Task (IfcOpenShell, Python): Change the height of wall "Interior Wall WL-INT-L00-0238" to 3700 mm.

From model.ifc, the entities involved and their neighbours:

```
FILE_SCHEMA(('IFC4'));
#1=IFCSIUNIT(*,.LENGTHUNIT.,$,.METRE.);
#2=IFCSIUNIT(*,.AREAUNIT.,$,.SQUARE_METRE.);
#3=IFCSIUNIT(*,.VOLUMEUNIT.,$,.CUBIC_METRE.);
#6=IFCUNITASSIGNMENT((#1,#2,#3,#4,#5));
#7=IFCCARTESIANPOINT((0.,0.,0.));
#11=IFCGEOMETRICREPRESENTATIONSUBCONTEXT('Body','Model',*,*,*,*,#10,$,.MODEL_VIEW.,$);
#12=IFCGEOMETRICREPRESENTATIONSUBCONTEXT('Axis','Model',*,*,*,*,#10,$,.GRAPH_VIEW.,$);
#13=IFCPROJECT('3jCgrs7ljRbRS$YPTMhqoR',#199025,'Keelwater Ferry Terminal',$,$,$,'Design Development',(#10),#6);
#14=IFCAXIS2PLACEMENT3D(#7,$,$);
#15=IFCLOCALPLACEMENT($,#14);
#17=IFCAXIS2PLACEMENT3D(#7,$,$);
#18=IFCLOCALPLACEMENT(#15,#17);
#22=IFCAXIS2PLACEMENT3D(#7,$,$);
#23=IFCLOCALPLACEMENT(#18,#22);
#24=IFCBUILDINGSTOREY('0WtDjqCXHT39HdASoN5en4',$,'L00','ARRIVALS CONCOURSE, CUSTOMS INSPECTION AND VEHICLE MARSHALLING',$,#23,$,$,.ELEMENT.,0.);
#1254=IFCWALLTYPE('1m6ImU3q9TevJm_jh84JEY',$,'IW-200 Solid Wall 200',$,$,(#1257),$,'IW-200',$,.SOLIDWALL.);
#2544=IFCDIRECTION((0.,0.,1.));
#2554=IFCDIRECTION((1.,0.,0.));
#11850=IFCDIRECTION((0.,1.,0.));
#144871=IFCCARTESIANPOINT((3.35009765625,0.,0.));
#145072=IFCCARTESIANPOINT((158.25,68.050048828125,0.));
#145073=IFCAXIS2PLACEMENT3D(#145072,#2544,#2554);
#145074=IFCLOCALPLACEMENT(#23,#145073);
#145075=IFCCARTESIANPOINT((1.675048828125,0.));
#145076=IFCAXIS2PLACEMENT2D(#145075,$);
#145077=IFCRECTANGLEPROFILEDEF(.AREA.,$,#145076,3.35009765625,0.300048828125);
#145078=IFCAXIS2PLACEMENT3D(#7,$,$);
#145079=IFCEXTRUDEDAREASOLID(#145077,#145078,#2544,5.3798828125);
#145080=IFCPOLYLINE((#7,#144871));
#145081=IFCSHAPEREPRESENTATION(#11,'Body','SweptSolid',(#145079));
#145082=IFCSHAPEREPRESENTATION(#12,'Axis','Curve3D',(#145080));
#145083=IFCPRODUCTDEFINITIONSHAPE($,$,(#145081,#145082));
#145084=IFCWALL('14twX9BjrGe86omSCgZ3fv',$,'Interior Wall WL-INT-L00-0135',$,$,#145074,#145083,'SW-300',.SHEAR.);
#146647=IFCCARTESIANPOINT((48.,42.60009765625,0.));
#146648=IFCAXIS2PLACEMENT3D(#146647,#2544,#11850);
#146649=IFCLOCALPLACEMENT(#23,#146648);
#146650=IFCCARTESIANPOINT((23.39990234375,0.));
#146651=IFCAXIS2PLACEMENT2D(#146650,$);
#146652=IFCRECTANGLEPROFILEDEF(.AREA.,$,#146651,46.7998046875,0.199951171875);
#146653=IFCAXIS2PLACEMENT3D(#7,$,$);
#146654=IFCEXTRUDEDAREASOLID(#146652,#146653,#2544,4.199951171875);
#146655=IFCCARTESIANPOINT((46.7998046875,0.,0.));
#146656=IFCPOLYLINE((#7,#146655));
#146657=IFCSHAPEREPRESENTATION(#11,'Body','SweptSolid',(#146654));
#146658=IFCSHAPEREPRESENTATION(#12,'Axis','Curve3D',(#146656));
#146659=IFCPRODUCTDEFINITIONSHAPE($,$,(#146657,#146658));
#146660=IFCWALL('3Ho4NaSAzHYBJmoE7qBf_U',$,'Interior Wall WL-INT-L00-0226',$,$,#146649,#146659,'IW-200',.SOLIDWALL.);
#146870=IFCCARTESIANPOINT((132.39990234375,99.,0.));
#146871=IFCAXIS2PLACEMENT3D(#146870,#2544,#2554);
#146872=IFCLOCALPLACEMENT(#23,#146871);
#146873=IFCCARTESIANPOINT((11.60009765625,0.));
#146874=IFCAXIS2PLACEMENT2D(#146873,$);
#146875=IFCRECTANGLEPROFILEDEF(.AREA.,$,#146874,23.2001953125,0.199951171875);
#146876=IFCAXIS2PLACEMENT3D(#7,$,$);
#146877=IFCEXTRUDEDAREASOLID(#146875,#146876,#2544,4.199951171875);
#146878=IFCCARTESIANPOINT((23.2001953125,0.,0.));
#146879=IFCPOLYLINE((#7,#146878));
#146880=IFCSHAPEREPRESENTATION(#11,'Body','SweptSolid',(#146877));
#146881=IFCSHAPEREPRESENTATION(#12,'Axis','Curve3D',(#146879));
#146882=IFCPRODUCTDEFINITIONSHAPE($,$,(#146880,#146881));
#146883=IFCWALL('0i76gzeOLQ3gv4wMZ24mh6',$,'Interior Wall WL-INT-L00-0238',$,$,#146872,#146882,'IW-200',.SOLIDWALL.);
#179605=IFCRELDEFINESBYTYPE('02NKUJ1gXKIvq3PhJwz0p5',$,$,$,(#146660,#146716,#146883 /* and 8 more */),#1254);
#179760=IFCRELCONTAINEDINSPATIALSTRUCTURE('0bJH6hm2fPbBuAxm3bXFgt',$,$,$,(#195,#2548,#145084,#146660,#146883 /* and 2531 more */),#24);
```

```python
import ifcopenshell
import ifcopenshell.geom
import ifcopenshell.util.representation
import ifcopenshell.util.shape
import ifcopenshell.util.unit

model = ifcopenshell.open("model.ifc")
unit_scale = ifcopenshell.util.unit.calculate_unit_scale(model)
settings = ifcopenshell.geom.settings()


def volume(element):
    """Net volume in cubic metres, openings subtracted."""
    shape = ifcopenshell.geom.create_shape(settings, element)
    return ifcopenshell.util.shape.get_volume(shape.geometry)


wall = model.by_guid("0i76gzeOLQ3gv4wMZ24mh6")
before = volume(wall)

body = ifcopenshell.util.representation.get_representation(wall, "Model", "Body")
solid = body.Items[0]
old_height = solid.Depth
solid.Depth = 3.7 / unit_scale
after = volume(wall)

print(f"height {old_height:g} -> {solid.Depth:g}, volume {before:.3f} -> {after:.3f} m3")

model.write("model_v2.ifc")
```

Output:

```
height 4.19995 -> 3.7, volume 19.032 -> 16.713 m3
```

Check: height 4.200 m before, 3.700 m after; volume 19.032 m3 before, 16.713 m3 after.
